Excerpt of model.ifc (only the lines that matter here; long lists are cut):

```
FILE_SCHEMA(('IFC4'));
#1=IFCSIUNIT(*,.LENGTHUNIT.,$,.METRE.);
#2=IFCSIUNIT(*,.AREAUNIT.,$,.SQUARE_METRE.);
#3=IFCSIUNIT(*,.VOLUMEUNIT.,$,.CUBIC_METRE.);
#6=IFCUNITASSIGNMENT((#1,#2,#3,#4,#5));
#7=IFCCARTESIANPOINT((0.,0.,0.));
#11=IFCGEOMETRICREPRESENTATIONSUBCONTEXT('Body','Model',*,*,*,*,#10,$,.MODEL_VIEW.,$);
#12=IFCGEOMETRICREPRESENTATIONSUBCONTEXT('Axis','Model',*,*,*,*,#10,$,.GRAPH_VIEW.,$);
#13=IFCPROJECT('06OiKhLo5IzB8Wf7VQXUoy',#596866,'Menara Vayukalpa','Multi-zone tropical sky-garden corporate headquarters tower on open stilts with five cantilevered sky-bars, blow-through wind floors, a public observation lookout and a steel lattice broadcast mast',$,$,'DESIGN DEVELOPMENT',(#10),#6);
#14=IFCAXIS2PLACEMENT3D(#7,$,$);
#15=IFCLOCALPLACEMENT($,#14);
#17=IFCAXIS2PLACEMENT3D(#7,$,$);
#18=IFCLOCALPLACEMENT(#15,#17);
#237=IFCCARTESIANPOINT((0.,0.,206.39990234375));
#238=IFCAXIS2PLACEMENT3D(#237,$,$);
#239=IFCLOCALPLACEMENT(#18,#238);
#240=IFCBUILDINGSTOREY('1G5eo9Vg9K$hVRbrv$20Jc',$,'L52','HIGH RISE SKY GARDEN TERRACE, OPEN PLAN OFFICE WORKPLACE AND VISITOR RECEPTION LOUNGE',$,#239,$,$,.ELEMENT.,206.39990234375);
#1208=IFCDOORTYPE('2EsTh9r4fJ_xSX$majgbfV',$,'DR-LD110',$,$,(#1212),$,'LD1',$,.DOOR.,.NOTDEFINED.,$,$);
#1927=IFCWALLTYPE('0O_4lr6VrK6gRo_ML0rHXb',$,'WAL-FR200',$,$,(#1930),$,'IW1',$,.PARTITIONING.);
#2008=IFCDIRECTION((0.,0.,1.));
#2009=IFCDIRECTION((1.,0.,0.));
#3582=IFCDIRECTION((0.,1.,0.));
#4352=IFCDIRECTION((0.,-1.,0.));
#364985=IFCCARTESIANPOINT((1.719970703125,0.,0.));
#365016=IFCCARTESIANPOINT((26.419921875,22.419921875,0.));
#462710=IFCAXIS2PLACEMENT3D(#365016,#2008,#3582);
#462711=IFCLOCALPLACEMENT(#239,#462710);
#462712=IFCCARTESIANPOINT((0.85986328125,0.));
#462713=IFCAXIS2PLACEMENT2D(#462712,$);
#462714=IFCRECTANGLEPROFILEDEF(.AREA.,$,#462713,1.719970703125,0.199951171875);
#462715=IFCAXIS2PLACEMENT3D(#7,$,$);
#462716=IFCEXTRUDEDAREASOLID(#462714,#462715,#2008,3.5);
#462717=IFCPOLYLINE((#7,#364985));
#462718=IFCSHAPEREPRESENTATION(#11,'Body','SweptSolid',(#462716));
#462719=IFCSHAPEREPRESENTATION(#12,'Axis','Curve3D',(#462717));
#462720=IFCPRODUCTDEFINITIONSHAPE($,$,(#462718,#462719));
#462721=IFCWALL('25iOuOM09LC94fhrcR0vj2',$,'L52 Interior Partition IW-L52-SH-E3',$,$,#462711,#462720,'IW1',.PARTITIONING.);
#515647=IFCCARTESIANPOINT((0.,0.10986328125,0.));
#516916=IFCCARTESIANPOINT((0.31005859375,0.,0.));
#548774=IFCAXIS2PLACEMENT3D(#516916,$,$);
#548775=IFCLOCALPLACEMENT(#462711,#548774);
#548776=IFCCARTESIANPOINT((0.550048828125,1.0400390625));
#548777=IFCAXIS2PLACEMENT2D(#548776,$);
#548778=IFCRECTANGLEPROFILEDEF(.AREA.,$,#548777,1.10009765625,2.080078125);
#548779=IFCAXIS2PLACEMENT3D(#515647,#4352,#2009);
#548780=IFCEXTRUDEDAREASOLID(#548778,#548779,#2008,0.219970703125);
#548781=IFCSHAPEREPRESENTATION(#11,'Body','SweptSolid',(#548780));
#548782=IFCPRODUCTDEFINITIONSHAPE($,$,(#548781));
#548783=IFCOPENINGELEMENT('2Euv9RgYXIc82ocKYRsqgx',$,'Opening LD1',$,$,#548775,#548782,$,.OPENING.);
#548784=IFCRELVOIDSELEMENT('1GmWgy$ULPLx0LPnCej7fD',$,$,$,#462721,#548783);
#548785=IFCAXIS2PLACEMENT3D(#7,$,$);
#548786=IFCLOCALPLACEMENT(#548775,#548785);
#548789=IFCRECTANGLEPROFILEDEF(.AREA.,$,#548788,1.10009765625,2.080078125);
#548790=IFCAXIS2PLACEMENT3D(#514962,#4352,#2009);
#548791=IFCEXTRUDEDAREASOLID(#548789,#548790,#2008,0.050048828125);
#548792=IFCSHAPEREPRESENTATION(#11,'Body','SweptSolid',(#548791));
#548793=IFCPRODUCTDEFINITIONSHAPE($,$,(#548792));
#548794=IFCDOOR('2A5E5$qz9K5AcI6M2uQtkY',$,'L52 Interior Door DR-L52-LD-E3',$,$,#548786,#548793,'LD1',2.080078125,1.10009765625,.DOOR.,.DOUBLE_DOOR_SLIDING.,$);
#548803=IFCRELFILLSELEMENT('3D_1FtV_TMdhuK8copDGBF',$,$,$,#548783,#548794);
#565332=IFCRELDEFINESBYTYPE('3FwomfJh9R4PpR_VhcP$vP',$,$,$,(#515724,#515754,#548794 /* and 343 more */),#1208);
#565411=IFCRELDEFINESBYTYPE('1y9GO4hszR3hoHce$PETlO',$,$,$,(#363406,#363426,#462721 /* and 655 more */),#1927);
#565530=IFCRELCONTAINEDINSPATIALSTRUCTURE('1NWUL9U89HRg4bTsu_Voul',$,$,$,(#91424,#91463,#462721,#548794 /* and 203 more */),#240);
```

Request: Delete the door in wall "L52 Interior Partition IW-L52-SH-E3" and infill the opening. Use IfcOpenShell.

```python
import ifcopenshell
import ifcopenshell.api.feature
import ifcopenshell.api.root
import ifcopenshell.geom
import ifcopenshell.util.shape

model = ifcopenshell.open("model.ifc")
settings = ifcopenshell.geom.settings()


def volume(element):
    """Net volume in cubic metres, openings subtracted."""
    shape = ifcopenshell.geom.create_shape(settings, element)
    return ifcopenshell.util.shape.get_volume(shape.geometry)


door = model.by_id(548794)
opening = door.FillsVoids[0].RelatingOpeningElement
wall = opening.VoidsElements[0].RelatingBuildingElement
before = volume(wall)

ifcopenshell.api.root.remove_product(model, product=door)
ifcopenshell.api.feature.remove_feature(model, feature=opening)

after = volume(wall)

print(f"wall volume {before:.3f} -> {after:.3f} m3")

model.write("model_edited.ifc")
```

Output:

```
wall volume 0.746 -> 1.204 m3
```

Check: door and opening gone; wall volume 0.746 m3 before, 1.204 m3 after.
